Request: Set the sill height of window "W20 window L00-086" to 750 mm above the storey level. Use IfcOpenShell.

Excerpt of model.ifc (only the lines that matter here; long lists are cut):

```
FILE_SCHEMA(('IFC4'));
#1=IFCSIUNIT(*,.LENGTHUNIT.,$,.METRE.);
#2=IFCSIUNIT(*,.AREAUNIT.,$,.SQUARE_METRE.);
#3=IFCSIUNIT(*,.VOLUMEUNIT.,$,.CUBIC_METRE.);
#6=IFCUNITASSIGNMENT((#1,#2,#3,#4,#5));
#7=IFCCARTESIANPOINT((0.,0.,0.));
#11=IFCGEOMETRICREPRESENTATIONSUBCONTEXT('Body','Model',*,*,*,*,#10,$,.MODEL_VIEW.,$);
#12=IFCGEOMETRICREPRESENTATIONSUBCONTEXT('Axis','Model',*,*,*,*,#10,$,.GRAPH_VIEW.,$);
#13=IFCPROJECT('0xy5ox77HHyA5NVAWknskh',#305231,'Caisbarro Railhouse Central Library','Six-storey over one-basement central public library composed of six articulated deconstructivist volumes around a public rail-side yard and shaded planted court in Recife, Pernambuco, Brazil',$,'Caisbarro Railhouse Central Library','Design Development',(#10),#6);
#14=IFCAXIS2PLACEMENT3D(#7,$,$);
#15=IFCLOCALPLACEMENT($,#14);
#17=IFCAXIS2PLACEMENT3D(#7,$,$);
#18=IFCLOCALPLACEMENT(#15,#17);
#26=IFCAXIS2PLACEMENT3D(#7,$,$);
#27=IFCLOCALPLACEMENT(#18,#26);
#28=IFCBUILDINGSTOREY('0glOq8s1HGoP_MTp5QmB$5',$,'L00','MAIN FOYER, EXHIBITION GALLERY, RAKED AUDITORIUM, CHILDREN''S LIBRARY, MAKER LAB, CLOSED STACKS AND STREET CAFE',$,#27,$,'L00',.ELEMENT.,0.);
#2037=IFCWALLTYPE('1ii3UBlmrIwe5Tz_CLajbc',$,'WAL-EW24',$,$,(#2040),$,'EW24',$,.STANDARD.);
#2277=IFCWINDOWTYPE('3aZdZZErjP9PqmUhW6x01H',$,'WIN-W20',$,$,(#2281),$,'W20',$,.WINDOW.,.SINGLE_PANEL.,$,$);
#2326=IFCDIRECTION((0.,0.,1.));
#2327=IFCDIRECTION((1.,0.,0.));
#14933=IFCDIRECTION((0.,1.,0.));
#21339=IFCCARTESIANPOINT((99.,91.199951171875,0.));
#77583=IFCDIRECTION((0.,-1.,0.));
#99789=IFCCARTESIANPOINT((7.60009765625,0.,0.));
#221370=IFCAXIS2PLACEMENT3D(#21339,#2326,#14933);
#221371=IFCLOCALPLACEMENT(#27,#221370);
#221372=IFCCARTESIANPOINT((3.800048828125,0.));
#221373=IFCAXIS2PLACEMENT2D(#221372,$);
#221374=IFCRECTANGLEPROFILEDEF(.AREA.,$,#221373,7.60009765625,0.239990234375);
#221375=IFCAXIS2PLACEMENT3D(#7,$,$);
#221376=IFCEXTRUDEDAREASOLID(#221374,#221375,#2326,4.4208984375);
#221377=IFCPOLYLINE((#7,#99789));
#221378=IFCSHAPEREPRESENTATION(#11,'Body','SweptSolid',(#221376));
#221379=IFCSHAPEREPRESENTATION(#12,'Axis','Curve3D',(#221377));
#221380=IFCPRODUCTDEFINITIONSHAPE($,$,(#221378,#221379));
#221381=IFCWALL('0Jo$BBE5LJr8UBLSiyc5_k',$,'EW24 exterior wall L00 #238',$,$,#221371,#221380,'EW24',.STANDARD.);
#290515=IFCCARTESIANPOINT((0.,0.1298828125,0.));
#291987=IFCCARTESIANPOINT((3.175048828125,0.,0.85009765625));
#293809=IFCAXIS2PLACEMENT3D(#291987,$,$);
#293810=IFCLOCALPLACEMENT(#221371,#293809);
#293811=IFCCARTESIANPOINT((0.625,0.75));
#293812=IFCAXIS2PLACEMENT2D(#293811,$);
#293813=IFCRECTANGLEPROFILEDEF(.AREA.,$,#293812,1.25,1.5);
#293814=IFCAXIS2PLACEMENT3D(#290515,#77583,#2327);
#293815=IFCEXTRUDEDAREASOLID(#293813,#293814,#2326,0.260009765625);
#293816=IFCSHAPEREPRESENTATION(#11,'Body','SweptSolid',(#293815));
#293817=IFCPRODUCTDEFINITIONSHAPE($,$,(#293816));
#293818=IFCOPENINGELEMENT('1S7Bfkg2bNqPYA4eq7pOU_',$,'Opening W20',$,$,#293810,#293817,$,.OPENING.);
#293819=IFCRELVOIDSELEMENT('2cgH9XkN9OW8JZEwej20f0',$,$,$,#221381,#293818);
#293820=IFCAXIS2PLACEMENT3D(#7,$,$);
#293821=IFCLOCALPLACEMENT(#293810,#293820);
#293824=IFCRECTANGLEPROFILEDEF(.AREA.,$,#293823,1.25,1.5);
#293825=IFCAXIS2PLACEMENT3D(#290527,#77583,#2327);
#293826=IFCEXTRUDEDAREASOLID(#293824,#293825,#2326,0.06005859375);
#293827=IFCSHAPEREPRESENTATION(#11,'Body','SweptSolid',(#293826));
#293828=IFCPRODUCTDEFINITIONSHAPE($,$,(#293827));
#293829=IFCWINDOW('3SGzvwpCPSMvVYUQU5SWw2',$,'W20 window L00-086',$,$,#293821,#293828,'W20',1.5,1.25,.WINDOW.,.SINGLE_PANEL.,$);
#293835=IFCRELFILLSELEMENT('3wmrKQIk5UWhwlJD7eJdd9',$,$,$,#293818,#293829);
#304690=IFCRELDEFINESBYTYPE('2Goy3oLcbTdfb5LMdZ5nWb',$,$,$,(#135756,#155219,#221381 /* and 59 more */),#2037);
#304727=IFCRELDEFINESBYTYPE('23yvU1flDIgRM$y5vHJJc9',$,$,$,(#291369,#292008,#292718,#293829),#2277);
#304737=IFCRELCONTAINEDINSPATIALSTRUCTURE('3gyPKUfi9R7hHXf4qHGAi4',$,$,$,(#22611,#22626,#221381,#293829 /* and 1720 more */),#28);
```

```python
import numpy as np
import ifcopenshell
import ifcopenshell.api.geometry
import ifcopenshell.geom
import ifcopenshell.util.element
import ifcopenshell.util.placement
import ifcopenshell.util.shape
import ifcopenshell.util.unit

model = ifcopenshell.open("model.ifc")
unit_scale = ifcopenshell.util.unit.calculate_unit_scale(model)

window = model.by_guid("3SGzvwpCPSMvVYUQU5SWw2")
opening = window.FillsVoids[0].RelatingOpeningElement
storey = ifcopenshell.util.element.get_container(window, ifc_class="IfcBuildingStorey")
level = ifcopenshell.util.placement.get_local_placement(storey.ObjectPlacement)[2, 3]

# The opening's origin need not be at the sill, so measure its lowest point.
shape = ifcopenshell.geom.create_shape(ifcopenshell.geom.settings(), opening)
bottom = ifcopenshell.util.shape.get_shape_bottom_elevation(shape, shape.geometry) / unit_scale
dz = level + 0.75 - bottom

shift = np.array([0.0, 0.0, dz])
# The window is placed relative to its opening, so it follows when the opening moves.
matrix = ifcopenshell.util.placement.get_local_placement(opening.ObjectPlacement)
matrix[:3, 3] += shift
ifcopenshell.api.geometry.edit_object_placement(
    model, product=opening, matrix=matrix, is_si=False, should_transform_children=True
)

print(f"moved by {dz * unit_scale:+.3f} m")

model.write("model_edited.ifc")
```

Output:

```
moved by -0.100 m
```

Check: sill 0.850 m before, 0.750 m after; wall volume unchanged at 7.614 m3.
